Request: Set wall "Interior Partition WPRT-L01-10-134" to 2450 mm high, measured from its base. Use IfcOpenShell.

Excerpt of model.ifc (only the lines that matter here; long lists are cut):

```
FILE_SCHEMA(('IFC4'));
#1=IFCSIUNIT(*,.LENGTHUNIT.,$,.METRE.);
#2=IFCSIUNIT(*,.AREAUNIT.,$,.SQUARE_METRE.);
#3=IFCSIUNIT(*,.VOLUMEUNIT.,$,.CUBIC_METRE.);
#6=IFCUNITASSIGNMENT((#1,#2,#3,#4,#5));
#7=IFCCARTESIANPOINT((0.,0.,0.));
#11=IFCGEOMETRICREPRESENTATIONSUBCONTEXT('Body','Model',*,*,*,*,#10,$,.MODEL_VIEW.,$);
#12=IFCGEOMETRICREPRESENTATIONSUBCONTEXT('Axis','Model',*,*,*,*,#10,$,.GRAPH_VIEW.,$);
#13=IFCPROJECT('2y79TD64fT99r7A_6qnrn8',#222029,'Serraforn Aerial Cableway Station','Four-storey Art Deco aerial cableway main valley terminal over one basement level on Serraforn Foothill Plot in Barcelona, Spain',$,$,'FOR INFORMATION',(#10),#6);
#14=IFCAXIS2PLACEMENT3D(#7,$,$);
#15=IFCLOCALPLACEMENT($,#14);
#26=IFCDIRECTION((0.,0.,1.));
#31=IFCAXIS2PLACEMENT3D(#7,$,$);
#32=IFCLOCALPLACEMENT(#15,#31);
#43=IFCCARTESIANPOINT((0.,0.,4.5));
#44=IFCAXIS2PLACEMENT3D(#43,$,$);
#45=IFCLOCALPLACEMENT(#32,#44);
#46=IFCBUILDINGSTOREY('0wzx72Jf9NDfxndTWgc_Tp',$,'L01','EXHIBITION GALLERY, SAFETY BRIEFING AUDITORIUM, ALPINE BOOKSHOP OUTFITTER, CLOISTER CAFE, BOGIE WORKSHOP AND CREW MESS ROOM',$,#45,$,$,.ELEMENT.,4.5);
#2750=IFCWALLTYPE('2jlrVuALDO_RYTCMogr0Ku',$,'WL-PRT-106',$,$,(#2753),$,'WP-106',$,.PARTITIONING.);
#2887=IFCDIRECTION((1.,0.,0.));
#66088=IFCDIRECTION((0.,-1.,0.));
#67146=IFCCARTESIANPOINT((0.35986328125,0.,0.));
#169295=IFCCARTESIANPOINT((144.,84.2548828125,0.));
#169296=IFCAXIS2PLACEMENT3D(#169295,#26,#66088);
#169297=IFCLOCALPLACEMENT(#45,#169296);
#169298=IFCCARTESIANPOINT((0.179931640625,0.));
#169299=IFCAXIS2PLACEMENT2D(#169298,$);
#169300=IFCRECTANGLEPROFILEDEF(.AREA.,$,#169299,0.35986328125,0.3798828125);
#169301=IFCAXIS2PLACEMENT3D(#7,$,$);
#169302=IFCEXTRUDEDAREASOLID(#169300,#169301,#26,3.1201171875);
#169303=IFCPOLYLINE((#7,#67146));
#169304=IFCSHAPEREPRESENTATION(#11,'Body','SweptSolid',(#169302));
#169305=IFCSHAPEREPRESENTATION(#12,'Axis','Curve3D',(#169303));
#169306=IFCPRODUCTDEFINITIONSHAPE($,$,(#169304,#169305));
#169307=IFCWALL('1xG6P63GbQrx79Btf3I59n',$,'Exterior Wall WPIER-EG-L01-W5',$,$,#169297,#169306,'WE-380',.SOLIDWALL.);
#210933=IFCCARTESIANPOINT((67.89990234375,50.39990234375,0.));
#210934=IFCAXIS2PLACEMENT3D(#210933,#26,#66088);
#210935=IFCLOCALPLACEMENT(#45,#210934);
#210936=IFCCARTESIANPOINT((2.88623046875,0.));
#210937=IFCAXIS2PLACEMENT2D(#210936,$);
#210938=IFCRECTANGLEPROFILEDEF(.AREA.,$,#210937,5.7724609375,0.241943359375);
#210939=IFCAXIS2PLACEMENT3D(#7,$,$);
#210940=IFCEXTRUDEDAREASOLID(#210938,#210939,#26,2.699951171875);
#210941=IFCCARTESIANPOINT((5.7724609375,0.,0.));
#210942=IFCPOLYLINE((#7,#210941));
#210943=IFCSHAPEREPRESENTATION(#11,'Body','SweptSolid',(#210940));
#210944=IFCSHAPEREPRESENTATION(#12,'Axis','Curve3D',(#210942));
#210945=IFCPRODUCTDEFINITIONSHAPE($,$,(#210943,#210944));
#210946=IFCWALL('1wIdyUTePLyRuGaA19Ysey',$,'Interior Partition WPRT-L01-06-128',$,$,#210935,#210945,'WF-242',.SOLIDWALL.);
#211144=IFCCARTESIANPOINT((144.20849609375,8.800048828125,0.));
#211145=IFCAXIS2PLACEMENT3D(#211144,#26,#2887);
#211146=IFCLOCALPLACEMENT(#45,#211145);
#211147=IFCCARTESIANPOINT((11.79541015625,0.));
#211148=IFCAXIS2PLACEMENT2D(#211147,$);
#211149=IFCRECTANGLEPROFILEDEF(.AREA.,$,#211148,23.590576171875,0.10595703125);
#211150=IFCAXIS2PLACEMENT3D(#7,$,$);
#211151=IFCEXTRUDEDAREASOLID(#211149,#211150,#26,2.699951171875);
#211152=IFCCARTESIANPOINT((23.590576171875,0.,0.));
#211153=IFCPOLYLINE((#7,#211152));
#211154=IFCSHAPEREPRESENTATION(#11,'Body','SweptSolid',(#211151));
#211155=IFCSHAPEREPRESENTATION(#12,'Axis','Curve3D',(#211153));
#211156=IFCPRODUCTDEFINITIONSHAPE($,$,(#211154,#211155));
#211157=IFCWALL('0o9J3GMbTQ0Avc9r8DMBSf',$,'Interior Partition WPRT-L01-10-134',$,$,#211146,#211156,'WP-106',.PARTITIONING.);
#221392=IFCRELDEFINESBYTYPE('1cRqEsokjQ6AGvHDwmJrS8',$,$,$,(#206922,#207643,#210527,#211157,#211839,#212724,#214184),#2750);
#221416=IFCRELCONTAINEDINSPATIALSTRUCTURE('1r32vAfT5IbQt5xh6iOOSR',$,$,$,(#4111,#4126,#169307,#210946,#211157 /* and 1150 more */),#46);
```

```python
import ifcopenshell
import ifcopenshell.geom
import ifcopenshell.util.representation
import ifcopenshell.util.shape
import ifcopenshell.util.unit

model = ifcopenshell.open("model.ifc")
unit_scale = ifcopenshell.util.unit.calculate_unit_scale(model)
settings = ifcopenshell.geom.settings()


def volume(element):
    """Net volume in cubic metres, openings subtracted."""
    shape = ifcopenshell.geom.create_shape(settings, element)
    return ifcopenshell.util.shape.get_volume(shape.geometry)


wall = model.by_guid("0o9J3GMbTQ0Avc9r8DMBSf")
before = volume(wall)

body = ifcopenshell.util.representation.get_representation(wall, "Model", "Body")
solid = body.Items[0]
old_height = solid.Depth
solid.Depth = 2.45 / unit_scale
after = volume(wall)

print(f"height {old_height:g} -> {solid.Depth:g}, volume {before:.3f} -> {after:.3f} m3")

model.write("model_edited.ifc")
```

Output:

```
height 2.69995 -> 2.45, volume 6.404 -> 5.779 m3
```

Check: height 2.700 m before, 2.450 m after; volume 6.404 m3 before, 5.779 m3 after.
